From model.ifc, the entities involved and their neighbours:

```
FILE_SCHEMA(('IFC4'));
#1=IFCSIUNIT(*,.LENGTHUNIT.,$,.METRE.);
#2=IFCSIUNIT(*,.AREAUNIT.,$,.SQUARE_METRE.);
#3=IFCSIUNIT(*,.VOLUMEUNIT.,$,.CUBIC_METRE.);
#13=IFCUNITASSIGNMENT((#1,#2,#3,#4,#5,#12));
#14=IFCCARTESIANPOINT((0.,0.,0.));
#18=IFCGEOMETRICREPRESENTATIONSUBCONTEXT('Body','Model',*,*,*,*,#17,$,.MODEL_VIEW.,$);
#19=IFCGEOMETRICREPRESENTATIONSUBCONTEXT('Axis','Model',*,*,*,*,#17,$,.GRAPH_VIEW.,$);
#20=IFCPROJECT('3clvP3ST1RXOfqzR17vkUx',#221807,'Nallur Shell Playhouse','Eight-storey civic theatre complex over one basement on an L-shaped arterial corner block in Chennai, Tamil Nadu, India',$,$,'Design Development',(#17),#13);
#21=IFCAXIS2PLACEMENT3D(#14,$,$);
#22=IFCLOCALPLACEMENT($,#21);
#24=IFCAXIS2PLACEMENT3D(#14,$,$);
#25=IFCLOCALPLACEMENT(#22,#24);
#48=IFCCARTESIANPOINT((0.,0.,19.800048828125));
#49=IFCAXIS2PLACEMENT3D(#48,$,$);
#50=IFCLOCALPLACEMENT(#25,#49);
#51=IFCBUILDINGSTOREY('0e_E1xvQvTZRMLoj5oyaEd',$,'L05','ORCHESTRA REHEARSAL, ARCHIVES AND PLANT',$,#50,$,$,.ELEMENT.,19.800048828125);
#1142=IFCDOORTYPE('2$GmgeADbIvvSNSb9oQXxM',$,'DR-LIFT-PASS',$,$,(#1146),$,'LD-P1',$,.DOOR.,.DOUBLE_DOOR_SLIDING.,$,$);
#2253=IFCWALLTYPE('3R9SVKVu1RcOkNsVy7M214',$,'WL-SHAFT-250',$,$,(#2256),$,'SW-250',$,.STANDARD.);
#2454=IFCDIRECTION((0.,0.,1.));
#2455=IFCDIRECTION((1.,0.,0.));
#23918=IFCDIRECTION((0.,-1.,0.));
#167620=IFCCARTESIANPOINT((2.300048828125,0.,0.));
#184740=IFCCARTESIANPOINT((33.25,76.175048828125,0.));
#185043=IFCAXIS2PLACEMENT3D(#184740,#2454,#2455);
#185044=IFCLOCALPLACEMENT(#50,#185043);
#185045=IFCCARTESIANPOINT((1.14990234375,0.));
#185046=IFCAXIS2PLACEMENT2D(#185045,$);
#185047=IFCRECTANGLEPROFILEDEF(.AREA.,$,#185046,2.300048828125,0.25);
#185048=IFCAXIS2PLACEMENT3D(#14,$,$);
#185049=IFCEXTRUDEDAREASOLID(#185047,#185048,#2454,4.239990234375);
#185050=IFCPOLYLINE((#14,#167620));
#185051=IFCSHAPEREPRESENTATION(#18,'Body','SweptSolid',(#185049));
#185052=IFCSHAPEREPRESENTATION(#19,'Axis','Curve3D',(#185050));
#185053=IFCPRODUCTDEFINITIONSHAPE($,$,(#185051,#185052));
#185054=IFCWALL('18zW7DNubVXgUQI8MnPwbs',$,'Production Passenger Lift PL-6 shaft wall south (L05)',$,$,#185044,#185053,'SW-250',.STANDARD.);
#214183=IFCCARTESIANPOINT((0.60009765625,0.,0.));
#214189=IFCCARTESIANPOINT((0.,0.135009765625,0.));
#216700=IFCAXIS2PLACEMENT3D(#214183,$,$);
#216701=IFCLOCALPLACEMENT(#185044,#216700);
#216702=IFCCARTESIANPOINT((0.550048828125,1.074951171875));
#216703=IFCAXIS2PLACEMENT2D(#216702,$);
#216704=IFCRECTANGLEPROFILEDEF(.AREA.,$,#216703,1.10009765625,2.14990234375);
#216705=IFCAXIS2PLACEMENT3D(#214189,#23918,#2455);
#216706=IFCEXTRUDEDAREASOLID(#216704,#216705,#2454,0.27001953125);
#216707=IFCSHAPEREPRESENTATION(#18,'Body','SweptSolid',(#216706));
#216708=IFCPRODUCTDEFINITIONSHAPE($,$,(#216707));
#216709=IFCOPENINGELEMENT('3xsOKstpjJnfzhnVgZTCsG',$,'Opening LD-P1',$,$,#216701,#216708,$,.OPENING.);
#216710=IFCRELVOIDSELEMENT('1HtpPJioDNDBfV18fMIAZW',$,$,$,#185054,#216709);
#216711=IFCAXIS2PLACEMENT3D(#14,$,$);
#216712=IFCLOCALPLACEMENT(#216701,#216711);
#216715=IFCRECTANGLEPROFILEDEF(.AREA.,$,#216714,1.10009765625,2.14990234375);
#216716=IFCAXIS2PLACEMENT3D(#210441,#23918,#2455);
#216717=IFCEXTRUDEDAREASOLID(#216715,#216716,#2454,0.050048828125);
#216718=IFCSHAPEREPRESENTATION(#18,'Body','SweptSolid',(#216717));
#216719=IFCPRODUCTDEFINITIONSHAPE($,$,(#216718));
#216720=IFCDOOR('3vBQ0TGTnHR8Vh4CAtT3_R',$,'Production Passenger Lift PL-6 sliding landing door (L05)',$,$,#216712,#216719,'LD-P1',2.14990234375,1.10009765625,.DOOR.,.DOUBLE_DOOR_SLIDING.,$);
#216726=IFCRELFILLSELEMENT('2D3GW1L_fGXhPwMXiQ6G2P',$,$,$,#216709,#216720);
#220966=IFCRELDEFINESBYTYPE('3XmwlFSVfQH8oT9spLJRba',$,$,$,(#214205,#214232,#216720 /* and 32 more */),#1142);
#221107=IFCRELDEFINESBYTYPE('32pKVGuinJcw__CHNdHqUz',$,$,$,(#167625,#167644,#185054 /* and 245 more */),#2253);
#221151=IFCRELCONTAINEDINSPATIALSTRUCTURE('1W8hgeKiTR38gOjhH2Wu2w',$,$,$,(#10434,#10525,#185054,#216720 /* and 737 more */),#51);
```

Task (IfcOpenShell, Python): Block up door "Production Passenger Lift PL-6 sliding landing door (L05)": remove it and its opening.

```python
import ifcopenshell
import ifcopenshell.api.feature
import ifcopenshell.api.root
import ifcopenshell.geom
import ifcopenshell.util.shape

model = ifcopenshell.open("model.ifc")
settings = ifcopenshell.geom.settings()


def volume(element):
    """Net volume in cubic metres, openings subtracted."""
    shape = ifcopenshell.geom.create_shape(settings, element)
    return ifcopenshell.util.shape.get_volume(shape.geometry)


door = model.by_guid("3vBQ0TGTnHR8Vh4CAtT3_R")
opening = door.FillsVoids[0].RelatingOpeningElement
wall = opening.VoidsElements[0].RelatingBuildingElement
before = volume(wall)

ifcopenshell.api.root.remove_product(model, product=door)
ifcopenshell.api.feature.remove_feature(model, feature=opening)

after = volume(wall)

print(f"wall volume {before:.3f} -> {after:.3f} m3")

model.write("model_edited.ifc")
```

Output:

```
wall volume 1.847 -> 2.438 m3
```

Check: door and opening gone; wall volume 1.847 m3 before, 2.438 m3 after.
